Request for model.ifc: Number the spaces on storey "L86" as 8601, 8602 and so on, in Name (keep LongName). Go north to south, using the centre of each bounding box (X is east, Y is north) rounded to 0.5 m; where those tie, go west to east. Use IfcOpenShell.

First a look at what the model holds.

```python
import ifcopenshell
import ifcopenshell.util.element
import ifcopenshell.util.placement

model = ifcopenshell.open("model.ifc")
print(model.schema)
storey = next(s for s in model.by_type("IfcBuildingStorey") if s.Name == "L86")
spaces = [e for e in ifcopenshell.util.element.get_decomposition(storey) if e.is_a("IfcSpace")]
for e in sorted(spaces, key=lambda e: e.id()):
    origin = ifcopenshell.util.placement.get_local_placement(e.ObjectPlacement)[:3, 3]
    print(e.id(), e.Name, e.LongName, origin.round(2) + 0.0, sep=" | ")
```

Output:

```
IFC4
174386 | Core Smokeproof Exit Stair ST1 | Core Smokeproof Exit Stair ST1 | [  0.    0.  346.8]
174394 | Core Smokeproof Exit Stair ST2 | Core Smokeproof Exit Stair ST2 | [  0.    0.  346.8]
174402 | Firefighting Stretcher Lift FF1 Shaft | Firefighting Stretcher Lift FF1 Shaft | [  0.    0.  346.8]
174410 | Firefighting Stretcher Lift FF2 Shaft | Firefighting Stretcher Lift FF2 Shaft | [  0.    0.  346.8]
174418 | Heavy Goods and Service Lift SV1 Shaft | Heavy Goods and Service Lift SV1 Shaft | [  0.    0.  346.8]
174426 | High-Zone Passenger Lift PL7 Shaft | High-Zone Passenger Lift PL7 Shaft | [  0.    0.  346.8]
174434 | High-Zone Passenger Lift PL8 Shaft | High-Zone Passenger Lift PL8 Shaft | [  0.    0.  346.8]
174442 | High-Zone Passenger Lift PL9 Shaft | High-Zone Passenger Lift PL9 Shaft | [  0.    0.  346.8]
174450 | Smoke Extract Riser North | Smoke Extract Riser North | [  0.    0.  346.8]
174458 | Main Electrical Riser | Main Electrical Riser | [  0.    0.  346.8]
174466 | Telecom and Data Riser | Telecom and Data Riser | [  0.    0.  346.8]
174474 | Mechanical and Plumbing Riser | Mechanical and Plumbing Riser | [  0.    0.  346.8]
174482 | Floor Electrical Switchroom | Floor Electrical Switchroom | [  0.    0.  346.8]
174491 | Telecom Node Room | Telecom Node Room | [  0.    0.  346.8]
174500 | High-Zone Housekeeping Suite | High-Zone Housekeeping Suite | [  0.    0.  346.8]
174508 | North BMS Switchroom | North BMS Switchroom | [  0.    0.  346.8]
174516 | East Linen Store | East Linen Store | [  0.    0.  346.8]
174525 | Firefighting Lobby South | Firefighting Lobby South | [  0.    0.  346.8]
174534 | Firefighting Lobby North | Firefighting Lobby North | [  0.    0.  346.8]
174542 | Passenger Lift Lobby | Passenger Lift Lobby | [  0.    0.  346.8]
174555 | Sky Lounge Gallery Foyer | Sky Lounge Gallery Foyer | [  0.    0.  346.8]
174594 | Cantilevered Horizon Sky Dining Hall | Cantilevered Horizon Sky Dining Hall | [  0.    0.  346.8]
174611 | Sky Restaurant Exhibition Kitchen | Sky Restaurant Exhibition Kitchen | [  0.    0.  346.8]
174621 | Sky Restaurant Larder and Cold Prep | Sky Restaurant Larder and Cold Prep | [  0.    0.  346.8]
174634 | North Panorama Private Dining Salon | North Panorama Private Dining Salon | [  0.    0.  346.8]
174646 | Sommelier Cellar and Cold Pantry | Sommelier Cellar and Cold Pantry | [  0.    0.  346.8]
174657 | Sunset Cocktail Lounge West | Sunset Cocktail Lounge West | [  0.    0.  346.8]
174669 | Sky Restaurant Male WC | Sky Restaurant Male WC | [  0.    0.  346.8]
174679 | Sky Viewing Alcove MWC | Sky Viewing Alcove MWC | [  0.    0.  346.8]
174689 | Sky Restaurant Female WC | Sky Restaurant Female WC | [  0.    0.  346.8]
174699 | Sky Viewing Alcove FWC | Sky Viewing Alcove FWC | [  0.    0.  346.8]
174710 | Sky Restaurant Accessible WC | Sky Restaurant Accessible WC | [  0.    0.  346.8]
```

```python
import ifcopenshell
import ifcopenshell.geom
import ifcopenshell.util.element
import ifcopenshell.util.shape

model = ifcopenshell.open("model.ifc")
settings = ifcopenshell.geom.settings()
settings.set("use-world-coords", True)


def centre(element):
    shape = ifcopenshell.geom.create_shape(settings, element)
    return ifcopenshell.util.shape.get_bbox_centroid(shape.geometry)


storey = next(s for s in model.by_type("IfcBuildingStorey") if s.Name == "L86")
spaces = [e for e in ifcopenshell.util.element.get_decomposition(storey) if e.is_a("IfcSpace")]

# Insertion points can sit at a corner or the storey origin, so sort by the geometry (in metres).
centres = {e: centre(e) for e in spaces}
spaces.sort(key=lambda e: (-round(centres[e][1] / 0.5), centres[e][0]))

for i, e in enumerate(spaces, start=1):
    number = f"86{i:02d}"
    e.Name = number
    print(e.id(), number)

model.write("model_rev.ifc")
```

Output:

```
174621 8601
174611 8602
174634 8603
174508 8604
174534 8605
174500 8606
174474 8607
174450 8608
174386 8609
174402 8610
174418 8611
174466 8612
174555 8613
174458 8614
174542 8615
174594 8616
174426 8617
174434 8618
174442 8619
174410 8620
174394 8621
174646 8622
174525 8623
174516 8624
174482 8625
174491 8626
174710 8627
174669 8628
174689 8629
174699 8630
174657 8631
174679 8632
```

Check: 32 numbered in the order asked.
